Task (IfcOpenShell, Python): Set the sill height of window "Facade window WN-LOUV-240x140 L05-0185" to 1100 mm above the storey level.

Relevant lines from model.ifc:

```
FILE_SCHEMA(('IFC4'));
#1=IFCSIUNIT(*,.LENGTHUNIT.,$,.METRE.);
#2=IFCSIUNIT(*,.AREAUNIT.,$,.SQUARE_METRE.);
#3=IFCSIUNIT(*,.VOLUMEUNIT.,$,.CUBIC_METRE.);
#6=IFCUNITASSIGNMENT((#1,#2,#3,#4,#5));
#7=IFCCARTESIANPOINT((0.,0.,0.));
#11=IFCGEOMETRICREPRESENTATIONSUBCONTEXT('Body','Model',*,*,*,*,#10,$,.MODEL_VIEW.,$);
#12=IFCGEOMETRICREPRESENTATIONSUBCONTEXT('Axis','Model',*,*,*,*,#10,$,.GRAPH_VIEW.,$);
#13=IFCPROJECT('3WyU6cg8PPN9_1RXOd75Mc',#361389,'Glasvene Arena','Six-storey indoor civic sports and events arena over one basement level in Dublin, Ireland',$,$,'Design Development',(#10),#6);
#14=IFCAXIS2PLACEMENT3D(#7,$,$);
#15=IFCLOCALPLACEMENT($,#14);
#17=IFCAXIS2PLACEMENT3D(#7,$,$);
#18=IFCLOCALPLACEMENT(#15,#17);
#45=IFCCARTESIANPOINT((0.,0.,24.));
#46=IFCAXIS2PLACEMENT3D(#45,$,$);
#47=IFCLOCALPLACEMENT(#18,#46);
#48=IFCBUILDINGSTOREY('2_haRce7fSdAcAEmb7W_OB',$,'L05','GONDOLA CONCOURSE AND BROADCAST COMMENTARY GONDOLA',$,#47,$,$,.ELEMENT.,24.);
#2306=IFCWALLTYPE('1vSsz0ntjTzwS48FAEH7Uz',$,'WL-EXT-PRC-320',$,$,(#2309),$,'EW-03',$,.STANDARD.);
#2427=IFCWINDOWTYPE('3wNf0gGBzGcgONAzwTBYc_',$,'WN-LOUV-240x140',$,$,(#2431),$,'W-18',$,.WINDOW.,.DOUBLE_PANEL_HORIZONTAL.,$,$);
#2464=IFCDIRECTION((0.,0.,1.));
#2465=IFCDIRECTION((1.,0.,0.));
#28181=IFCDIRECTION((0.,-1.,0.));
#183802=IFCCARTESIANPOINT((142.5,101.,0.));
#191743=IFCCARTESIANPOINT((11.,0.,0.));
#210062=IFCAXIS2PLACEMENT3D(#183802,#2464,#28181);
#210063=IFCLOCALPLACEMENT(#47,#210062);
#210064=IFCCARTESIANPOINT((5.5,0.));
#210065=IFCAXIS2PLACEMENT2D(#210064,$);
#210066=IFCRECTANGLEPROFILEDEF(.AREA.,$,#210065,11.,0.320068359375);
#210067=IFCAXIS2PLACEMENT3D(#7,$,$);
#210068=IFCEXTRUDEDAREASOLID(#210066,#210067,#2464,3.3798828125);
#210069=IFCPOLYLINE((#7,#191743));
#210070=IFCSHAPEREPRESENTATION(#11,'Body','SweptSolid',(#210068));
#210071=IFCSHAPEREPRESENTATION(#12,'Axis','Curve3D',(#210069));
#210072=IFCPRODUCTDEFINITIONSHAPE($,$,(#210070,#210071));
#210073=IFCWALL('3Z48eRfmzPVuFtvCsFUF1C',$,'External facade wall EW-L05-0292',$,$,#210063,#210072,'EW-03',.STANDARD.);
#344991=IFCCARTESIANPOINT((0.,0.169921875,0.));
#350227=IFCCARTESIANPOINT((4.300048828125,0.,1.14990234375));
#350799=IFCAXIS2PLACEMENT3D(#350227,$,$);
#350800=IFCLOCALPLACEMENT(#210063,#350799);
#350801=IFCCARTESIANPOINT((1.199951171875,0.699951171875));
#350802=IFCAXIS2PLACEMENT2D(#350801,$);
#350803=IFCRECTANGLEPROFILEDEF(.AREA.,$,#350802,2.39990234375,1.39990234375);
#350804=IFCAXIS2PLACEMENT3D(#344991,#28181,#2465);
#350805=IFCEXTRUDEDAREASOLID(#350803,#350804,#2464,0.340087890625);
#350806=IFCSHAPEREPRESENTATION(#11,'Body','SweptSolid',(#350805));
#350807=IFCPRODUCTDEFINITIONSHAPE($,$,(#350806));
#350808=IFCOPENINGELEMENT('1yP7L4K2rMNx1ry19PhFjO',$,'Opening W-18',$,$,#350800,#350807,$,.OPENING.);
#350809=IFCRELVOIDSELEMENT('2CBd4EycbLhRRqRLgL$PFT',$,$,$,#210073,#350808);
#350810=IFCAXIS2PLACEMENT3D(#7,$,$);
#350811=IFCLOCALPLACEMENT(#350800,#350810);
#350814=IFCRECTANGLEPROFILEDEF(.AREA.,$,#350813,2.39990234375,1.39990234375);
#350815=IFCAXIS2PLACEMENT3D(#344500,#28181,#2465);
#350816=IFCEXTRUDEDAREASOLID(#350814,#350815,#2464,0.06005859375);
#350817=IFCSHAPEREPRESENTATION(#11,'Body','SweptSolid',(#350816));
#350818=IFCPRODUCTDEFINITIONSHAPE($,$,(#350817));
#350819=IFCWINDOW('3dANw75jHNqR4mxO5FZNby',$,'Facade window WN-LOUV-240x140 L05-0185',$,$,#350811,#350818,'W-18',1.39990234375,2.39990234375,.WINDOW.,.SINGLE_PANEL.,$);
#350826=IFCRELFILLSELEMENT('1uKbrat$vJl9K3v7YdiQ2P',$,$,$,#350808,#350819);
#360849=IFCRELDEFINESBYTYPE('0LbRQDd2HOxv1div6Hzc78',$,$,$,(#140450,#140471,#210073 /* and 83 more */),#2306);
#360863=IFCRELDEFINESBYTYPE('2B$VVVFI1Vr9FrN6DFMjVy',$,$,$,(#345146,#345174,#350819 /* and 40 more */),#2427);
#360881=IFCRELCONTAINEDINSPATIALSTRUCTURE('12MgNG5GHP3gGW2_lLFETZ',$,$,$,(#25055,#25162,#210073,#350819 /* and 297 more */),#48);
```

```python
import numpy as np
import ifcopenshell
import ifcopenshell.api.geometry
import ifcopenshell.geom
import ifcopenshell.util.element
import ifcopenshell.util.placement
import ifcopenshell.util.shape
import ifcopenshell.util.unit

model = ifcopenshell.open("model.ifc")
unit_scale = ifcopenshell.util.unit.calculate_unit_scale(model)

window = model.by_guid("3dANw75jHNqR4mxO5FZNby")
opening = window.FillsVoids[0].RelatingOpeningElement
storey = ifcopenshell.util.element.get_container(window, ifc_class="IfcBuildingStorey")
level = ifcopenshell.util.placement.get_local_placement(storey.ObjectPlacement)[2, 3]

# The opening's origin need not be at the sill, so measure its lowest point.
shape = ifcopenshell.geom.create_shape(ifcopenshell.geom.settings(), opening)
bottom = ifcopenshell.util.shape.get_shape_bottom_elevation(shape, shape.geometry) / unit_scale
dz = level + 1.1 - bottom

shift = np.array([0.0, 0.0, dz])
# The window is placed relative to its opening, so it follows when the opening moves.
matrix = ifcopenshell.util.placement.get_local_placement(opening.ObjectPlacement)
matrix[:3, 3] += shift
ifcopenshell.api.geometry.edit_object_placement(
    model, product=opening, matrix=matrix, is_si=False, should_transform_children=True
)

print(f"moved by {dz * unit_scale:+.3f} m")

model.write("model_updated.ifc")
```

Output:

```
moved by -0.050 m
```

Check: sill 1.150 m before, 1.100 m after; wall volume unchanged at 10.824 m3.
